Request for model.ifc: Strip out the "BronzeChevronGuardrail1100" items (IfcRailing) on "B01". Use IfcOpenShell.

First a look at what the model holds.

```python
import ifcopenshell
import ifcopenshell.util.element

model = ifcopenshell.open("model.ifc")
print(model.schema)
storey = next(s for s in model.by_type("IfcBuildingStorey") if s.Name == "B01")
railings = [e for e in ifcopenshell.util.element.get_decomposition(storey) if e.is_a("IfcRailing")]
seen = {}
for e in railings:
    element_type = ifcopenshell.util.element.get_type(e)
    name = element_type.Name if element_type not in (None, e) else None
    seen[name] = seen.get(name, 0) + 1
for name, count in sorted(seen.items(), key=str):
    print(count, "x", name)
```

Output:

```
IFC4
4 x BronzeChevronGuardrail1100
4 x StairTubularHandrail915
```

```python
import ifcopenshell
import ifcopenshell.api.root
import ifcopenshell.util.element

model = ifcopenshell.open("model.ifc")

storey = next(s for s in model.by_type("IfcBuildingStorey") if s.Name == "B01")
railings = [e for e in ifcopenshell.util.element.get_decomposition(storey) if e.is_a("IfcRailing")]
targets = [e for e in railings if (t := ifcopenshell.util.element.get_type(e)) not in (None, e) and t.Name == "BronzeChevronGuardrail1100"]

for e in targets:
    ifcopenshell.api.root.remove_product(model, product=e)
print(len(targets), "removed")

model.write("model_rev.ifc")
```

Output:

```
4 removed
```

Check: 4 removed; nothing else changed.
